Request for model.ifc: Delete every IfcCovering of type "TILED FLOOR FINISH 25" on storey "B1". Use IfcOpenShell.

First a look at what the model holds.

```python
import ifcopenshell
import ifcopenshell.util.element

model = ifcopenshell.open("model.ifc")
print(model.schema)
storey = next(s for s in model.by_type("IfcBuildingStorey") if s.Name == "B1")
coverings = [e for e in ifcopenshell.util.element.get_decomposition(storey) if e.is_a("IfcCovering")]
seen = {}
for e in coverings:
    element_type = ifcopenshell.util.element.get_type(e)
    name = element_type.Name if element_type not in (None, e) else None
    seen[name] = seen.get(name, 0) + 1
for name, count in sorted(seen.items(), key=str):
    print(count, "x", name)
```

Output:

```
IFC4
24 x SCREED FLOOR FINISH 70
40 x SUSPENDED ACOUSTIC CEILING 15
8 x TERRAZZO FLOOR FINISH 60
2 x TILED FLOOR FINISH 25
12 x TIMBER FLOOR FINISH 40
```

```python
import ifcopenshell
import ifcopenshell.api.root
import ifcopenshell.util.element

model = ifcopenshell.open("model.ifc")

storey = next(s for s in model.by_type("IfcBuildingStorey") if s.Name == "B1")
coverings = [e for e in ifcopenshell.util.element.get_decomposition(storey) if e.is_a("IfcCovering")]
targets = [e for e in coverings if (t := ifcopenshell.util.element.get_type(e)) not in (None, e) and t.Name == "TILED FLOOR FINISH 25"]

for e in targets:
    ifcopenshell.api.root.remove_product(model, product=e)
print(len(targets), "removed")

model.write("model_v2.ifc")
```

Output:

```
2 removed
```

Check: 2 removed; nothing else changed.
